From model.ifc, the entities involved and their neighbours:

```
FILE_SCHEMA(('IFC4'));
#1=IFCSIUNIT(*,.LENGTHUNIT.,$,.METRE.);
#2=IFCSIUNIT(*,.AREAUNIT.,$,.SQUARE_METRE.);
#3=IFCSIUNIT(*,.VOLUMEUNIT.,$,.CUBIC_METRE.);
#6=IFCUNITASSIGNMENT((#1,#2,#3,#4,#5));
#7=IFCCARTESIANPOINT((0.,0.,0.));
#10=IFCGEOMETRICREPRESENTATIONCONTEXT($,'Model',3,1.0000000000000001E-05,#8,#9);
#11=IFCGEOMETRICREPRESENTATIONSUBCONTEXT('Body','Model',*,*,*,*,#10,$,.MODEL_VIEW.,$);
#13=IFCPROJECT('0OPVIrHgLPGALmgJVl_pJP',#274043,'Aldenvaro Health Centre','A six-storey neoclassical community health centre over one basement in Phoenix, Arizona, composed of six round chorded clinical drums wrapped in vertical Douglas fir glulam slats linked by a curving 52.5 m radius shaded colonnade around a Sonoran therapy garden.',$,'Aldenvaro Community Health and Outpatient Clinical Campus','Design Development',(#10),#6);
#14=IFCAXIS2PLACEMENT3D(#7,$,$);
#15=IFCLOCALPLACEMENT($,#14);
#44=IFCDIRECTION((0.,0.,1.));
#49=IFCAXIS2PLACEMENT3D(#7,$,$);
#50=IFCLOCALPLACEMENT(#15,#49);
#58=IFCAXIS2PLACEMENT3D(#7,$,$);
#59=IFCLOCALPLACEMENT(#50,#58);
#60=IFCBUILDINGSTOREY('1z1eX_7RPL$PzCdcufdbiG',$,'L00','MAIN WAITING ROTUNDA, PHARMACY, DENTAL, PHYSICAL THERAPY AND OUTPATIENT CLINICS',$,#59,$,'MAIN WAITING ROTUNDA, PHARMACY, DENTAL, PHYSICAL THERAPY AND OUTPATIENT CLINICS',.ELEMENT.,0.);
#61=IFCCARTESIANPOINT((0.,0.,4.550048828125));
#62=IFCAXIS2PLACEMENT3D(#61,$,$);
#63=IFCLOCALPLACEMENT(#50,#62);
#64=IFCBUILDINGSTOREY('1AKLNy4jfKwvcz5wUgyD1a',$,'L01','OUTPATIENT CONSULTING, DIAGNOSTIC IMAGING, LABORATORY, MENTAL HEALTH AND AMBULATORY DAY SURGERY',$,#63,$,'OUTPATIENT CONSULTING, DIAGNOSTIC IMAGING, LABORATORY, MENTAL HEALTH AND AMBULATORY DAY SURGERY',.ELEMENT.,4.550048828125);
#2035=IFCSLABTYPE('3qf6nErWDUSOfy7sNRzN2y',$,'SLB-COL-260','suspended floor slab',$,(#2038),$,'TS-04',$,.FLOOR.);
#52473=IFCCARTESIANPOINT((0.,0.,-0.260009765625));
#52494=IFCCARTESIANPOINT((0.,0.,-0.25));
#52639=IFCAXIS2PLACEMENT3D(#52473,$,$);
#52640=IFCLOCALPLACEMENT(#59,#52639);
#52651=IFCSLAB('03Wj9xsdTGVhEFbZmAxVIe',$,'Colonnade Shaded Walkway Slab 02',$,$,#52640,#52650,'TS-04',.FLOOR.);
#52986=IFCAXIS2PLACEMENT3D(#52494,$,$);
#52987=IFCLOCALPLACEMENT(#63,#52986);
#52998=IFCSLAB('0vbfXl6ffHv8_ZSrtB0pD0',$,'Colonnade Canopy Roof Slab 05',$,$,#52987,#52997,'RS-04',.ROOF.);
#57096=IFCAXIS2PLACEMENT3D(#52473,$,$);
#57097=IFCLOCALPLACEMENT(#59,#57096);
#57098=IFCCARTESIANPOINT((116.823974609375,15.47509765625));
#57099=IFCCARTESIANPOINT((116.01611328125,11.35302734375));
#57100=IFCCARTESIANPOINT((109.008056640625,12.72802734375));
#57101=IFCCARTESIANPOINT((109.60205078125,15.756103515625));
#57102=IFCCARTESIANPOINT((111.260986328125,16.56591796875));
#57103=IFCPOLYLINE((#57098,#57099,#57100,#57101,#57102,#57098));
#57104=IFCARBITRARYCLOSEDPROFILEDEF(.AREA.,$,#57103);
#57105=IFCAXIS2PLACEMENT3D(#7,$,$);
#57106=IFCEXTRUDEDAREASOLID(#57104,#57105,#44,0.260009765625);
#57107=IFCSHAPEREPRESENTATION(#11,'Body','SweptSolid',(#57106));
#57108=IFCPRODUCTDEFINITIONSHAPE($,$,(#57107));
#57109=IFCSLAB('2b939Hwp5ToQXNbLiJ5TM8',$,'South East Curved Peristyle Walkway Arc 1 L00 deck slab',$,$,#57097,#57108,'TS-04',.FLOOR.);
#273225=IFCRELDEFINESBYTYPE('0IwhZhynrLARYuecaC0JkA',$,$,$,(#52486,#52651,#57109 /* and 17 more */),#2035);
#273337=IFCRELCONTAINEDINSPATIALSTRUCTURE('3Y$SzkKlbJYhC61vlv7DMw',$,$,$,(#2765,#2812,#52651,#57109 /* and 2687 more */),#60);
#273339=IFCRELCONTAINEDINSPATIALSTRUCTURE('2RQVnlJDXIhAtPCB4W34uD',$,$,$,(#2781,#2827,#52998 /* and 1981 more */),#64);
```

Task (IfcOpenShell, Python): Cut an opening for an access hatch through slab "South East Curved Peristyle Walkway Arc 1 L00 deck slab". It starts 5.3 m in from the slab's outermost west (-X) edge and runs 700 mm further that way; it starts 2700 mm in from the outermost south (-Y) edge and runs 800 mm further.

```python
import numpy as np
import ifcopenshell
import ifcopenshell.api.feature
import ifcopenshell.api.geometry
import ifcopenshell.api.root
import ifcopenshell.geom
import ifcopenshell.util.placement
import ifcopenshell.util.representation
import ifcopenshell.util.shape
import ifcopenshell.util.unit

model = ifcopenshell.open("model.ifc")
unit_scale = ifcopenshell.util.unit.calculate_unit_scale(model)
settings = ifcopenshell.geom.settings()


def volume(element):
    """Net volume in cubic metres, openings subtracted."""
    shape = ifcopenshell.geom.create_shape(settings, element)
    return ifcopenshell.util.shape.get_volume(shape.geometry)


slab = model.by_guid("2b939Hwp5ToQXNbLiJ5TM8")
before = volume(slab)

# Extent in the slab's own axes, in metres. The edges named are its -X and -Y sides.
slab_shape = ifcopenshell.geom.create_shape(settings, slab)
vertices = ifcopenshell.util.shape.get_vertices(slab_shape.geometry)
x_min, y_min, bottom = vertices.min(axis=0)
top = vertices[:, 2].max()

opening = ifcopenshell.api.root.create_entity(model, ifc_class="IfcOpeningElement", name="Access hatch opening", predefined_type="OPENING")
context = ifcopenshell.util.representation.get_context(model, "Model", "Body", "MODEL_VIEW")
width, depth = 0.7, 0.8
outline = [(0.0, 0.0), (width, 0.0), (width, depth), (0.0, depth), (0.0, 0.0)]
# Overshoot both faces by 50 mm so the cut is clean.
shape = ifcopenshell.api.geometry.add_slab_representation(
    model, context=context, depth=top - bottom + 0.1, polyline=outline
)
ifcopenshell.api.geometry.assign_representation(model, product=opening, representation=shape)

matrix = ifcopenshell.util.placement.get_local_placement(slab.ObjectPlacement)
matrix[:, 3] = matrix @ np.append(np.array([x_min + 5.3, y_min + 2.7, bottom - 0.05]) / unit_scale, 1.0)
ifcopenshell.api.geometry.edit_object_placement(model, product=opening, matrix=matrix, is_si=False)
ifcopenshell.api.feature.add_feature(model, feature=opening, element=slab)

after = volume(slab)

print(f"slab volume {before:.3f} -> {after:.3f} m3")

model.write("model_rev.ifc")
```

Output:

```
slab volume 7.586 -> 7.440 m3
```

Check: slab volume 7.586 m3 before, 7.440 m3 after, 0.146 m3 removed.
